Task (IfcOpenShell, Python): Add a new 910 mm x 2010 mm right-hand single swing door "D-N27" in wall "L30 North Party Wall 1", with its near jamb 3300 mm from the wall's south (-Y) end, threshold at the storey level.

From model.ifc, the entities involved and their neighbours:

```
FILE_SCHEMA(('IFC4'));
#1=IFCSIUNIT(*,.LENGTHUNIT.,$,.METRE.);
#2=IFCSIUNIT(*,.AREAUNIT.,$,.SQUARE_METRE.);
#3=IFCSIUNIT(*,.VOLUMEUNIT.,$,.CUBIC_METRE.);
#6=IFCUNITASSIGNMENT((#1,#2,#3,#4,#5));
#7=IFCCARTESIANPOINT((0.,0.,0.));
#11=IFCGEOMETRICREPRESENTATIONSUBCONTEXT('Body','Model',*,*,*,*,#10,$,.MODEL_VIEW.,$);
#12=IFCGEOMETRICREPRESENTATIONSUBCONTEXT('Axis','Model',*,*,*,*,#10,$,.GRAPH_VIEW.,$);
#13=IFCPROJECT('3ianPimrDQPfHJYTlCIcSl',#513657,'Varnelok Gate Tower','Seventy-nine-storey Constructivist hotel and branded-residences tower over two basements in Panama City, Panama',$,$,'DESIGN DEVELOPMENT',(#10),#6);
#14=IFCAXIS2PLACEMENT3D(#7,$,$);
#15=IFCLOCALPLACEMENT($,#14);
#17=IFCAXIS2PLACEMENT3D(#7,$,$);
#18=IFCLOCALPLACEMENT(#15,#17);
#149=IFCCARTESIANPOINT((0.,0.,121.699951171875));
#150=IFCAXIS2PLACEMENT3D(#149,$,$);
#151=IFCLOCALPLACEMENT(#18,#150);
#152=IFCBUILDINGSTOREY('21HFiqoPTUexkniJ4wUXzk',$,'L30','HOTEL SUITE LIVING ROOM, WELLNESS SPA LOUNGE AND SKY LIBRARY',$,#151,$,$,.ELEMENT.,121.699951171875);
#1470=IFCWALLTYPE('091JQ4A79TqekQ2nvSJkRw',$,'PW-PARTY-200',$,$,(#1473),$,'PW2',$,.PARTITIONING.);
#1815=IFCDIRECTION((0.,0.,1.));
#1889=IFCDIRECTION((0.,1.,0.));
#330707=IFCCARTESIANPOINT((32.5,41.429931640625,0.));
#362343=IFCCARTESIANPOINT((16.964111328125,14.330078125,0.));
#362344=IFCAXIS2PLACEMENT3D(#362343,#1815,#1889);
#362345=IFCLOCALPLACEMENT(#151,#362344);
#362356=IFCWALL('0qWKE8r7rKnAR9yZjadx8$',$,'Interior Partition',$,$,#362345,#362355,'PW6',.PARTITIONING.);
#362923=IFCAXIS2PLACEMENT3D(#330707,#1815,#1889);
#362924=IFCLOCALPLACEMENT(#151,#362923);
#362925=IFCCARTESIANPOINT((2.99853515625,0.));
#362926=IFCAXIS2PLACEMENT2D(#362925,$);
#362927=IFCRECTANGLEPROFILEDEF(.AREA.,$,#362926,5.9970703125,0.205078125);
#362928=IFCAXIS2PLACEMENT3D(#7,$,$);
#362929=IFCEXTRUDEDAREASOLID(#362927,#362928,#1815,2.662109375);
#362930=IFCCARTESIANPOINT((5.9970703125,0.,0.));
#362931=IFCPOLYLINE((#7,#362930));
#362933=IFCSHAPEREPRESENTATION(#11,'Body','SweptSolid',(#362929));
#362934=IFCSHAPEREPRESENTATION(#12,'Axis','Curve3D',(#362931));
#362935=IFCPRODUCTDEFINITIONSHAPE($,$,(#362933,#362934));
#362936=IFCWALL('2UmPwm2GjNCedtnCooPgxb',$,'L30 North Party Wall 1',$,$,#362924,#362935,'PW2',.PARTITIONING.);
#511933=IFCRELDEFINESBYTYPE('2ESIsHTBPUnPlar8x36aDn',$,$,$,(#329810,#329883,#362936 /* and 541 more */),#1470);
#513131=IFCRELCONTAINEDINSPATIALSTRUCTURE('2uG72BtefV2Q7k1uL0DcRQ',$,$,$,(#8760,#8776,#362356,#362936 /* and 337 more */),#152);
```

```python
import numpy as np
import ifcopenshell
import ifcopenshell.api.feature
import ifcopenshell.api.geometry
import ifcopenshell.api.root
import ifcopenshell.api.spatial
import ifcopenshell.geom
import ifcopenshell.util.element
import ifcopenshell.util.placement
import ifcopenshell.util.representation
import ifcopenshell.util.shape
import ifcopenshell.util.unit

model = ifcopenshell.open("model.ifc")
unit_scale = ifcopenshell.util.unit.calculate_unit_scale(model)
settings = ifcopenshell.geom.settings()


def volume(element):
    """Net volume in cubic metres, openings subtracted."""
    shape = ifcopenshell.geom.create_shape(settings, element)
    return ifcopenshell.util.shape.get_volume(shape.geometry)


wall = model.by_guid("2UmPwm2GjNCedtnCooPgxb")
storey = ifcopenshell.util.element.get_container(wall, ifc_class="IfcBuildingStorey")
context = ifcopenshell.util.representation.get_context(model, "Model", "Body", "MODEL_VIEW")
before = volume(wall)

width, height, from_end, sill = 0.91, 2.01, 3.3, 0.0  # metres

# The wall runs along its own X axis, and the end named is its -X end.
wall_shape = ifcopenshell.geom.create_shape(settings, wall)
x, y, z = ifcopenshell.util.shape.get_vertices(wall_shape.geometry).T
start = x.min() + from_end
face, thickness = float(y.min()), float(y.max() - y.min())
wall_matrix = ifcopenshell.util.placement.get_local_placement(wall.ObjectPlacement)
level = ifcopenshell.util.placement.get_local_placement(storey.ObjectPlacement)[2, 3]


def in_wall(x, y):
    """Placement at x, y metres in the wall's axes, at sill height."""
    matrix = wall_matrix.copy()
    matrix[:, 3] = wall_matrix @ np.array([x / unit_scale, y / unit_scale, 0.0, 1.0])
    matrix[2, 3] = level + sill / unit_scale
    return matrix


# Opening: a box that overshoots both wall faces by 50 mm.
opening = ifcopenshell.api.root.create_entity(model, ifc_class="IfcOpeningElement", predefined_type="OPENING")
box = ifcopenshell.api.geometry.add_wall_representation(
    model, context=context, length=width, height=height, thickness=thickness + 0.1
)
ifcopenshell.api.geometry.assign_representation(model, product=opening, representation=box)
ifcopenshell.api.geometry.edit_object_placement(model, product=opening, matrix=in_wall(start, face - 0.05), is_si=False)
ifcopenshell.api.feature.add_feature(model, feature=opening, element=wall)

door = ifcopenshell.api.root.create_entity(model, ifc_class="IfcDoor", name="D-N27", predefined_type="DOOR")
door.OverallWidth, door.OverallHeight = width / unit_scale, height / unit_scale
door.OperationType = "SINGLE_SWING_RIGHT"
body = ifcopenshell.api.geometry.add_door_representation(
    model,
    context=context,
    overall_width=door.OverallWidth,
    overall_height=door.OverallHeight,
    operation_type="SINGLE_SWING_RIGHT",
    lining_properties={"LiningDepth": thickness / unit_scale, "ThresholdDepth": thickness / unit_scale},
)
ifcopenshell.api.geometry.assign_representation(model, product=door, representation=body)
ifcopenshell.api.spatial.assign_container(model, products=[door], relating_structure=storey)
ifcopenshell.api.feature.add_filling(model, opening=opening, element=door)

# The lining spans the wall, so the door starts at the wall face.
ifcopenshell.api.geometry.edit_object_placement(model, product=door, matrix=in_wall(start, face), is_si=False)

after = volume(wall)

print(f"wall volume {before:.3f} -> {after:.3f} m3")

model.write("model_edited.ifc")
```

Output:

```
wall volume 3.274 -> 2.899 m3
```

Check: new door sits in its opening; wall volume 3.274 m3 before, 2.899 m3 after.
